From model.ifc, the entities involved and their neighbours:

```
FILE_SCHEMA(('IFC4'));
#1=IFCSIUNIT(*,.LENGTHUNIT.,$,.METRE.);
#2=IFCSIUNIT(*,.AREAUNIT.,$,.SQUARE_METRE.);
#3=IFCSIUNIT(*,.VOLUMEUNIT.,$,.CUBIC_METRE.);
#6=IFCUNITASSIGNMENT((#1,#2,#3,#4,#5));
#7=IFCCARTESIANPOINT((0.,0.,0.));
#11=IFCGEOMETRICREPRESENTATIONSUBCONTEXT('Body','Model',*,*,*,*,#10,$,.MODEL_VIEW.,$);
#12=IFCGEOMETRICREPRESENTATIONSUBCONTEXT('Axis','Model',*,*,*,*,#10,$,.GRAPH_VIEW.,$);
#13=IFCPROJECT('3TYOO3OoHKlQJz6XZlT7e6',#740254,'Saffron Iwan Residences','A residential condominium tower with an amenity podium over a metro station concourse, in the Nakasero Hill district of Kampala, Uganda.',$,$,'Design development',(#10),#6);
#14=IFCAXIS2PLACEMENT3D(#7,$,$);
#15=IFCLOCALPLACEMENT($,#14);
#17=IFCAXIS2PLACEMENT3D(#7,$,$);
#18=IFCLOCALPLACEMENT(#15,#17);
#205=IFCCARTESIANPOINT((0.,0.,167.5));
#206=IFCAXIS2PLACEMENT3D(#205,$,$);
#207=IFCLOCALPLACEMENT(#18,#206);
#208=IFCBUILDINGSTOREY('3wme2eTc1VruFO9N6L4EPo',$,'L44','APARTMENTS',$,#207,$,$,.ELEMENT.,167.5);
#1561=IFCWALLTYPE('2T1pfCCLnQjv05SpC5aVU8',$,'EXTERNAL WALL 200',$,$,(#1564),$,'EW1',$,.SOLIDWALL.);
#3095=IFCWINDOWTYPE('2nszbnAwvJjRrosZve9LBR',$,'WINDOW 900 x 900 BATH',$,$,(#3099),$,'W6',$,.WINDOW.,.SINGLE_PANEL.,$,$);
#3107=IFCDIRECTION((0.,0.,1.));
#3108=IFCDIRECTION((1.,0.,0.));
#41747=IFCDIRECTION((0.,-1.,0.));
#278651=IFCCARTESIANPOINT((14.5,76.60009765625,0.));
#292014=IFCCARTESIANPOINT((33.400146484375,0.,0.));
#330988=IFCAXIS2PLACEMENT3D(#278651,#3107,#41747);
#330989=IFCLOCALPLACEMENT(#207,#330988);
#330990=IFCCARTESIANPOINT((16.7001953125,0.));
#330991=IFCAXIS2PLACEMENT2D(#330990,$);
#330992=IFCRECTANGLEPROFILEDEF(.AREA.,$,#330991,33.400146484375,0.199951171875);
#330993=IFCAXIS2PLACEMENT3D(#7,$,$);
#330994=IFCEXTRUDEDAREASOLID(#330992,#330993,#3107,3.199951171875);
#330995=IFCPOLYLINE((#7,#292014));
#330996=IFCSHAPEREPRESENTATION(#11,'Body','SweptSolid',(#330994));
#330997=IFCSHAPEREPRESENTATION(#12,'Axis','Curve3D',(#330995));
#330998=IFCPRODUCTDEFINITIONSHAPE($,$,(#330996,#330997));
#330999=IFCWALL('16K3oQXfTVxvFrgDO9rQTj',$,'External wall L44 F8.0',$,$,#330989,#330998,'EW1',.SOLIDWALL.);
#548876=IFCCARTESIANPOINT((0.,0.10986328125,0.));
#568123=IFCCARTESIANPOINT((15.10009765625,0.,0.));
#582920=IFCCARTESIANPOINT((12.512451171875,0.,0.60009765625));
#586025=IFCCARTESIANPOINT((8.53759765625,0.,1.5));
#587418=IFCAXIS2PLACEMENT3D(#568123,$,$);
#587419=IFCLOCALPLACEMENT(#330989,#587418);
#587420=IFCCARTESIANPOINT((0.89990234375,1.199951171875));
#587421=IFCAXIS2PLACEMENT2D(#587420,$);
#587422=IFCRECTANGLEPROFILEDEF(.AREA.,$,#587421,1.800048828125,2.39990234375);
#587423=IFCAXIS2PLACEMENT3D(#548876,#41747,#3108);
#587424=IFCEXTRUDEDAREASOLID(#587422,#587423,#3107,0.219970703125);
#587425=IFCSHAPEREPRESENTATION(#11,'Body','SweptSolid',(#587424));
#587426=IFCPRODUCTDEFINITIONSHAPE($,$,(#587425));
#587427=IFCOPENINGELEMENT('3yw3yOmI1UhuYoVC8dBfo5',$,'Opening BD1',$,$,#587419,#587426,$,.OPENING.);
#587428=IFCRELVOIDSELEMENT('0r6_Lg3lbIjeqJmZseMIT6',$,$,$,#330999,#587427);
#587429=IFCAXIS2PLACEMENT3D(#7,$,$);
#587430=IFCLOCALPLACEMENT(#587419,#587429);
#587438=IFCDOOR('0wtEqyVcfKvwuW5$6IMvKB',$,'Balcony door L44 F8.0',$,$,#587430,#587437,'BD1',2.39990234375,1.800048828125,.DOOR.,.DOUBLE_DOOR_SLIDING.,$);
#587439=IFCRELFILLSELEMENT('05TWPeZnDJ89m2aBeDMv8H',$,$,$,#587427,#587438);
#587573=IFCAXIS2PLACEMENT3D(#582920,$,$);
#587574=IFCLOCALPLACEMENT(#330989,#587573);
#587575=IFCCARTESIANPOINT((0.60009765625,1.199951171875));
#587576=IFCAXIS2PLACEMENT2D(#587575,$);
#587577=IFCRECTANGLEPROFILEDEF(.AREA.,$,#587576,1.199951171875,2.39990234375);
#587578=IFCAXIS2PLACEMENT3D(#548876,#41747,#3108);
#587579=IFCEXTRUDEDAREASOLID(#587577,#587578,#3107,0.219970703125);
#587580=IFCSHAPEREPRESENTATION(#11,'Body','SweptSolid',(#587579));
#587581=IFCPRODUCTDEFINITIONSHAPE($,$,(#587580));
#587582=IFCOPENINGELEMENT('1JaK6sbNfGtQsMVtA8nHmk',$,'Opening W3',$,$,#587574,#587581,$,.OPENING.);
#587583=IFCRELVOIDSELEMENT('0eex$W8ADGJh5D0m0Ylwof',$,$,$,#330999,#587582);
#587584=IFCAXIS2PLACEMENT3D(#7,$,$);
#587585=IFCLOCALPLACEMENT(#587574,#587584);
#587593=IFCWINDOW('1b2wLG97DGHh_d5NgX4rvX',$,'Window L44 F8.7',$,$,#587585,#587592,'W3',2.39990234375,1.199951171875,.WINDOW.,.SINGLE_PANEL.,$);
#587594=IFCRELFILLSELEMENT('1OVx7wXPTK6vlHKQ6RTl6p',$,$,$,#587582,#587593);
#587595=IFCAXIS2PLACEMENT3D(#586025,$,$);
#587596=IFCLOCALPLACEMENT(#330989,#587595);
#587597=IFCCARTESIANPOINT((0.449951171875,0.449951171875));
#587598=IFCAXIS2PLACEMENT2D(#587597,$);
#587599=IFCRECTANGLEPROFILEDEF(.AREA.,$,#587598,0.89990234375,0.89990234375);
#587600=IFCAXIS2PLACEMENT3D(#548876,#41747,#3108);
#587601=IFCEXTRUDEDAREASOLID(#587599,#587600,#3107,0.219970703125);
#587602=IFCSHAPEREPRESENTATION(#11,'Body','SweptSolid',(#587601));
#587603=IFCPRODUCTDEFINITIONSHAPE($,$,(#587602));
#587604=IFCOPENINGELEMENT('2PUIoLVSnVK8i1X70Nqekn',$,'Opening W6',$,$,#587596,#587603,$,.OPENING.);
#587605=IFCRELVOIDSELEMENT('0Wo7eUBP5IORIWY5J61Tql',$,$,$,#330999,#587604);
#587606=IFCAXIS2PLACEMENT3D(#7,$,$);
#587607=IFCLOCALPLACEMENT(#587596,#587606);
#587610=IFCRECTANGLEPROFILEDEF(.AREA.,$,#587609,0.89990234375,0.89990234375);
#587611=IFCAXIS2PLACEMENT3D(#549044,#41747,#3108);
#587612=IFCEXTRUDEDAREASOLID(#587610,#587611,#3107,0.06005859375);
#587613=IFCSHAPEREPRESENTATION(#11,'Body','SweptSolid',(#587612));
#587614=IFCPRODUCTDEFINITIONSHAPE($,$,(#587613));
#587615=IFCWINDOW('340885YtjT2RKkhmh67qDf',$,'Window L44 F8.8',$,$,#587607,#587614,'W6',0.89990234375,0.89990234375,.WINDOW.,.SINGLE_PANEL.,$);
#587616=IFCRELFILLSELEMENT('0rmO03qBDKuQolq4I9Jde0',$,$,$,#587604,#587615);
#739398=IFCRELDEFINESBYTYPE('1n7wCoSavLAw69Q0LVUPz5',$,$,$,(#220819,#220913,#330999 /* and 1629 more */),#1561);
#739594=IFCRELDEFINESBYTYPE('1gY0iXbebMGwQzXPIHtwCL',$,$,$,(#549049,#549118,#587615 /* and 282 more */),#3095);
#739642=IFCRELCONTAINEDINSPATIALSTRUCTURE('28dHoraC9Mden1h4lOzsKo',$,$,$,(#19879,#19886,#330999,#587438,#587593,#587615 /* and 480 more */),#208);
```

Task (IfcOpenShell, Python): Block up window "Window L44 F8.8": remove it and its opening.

```python
import ifcopenshell
import ifcopenshell.api.feature
import ifcopenshell.api.root
import ifcopenshell.geom
import ifcopenshell.util.shape

model = ifcopenshell.open("model.ifc")
settings = ifcopenshell.geom.settings()


def volume(element):
    """Net volume in cubic metres, openings subtracted."""
    shape = ifcopenshell.geom.create_shape(settings, element)
    return ifcopenshell.util.shape.get_volume(shape.geometry)


window = model.by_id(587615)
opening = window.FillsVoids[0].RelatingOpeningElement
wall = opening.VoidsElements[0].RelatingBuildingElement
before = volume(wall)

ifcopenshell.api.root.remove_product(model, product=window)
ifcopenshell.api.feature.remove_feature(model, feature=opening)

after = volume(wall)

print(f"wall volume {before:.3f} -> {after:.3f} m3")

model.write("model_v2.ifc")
```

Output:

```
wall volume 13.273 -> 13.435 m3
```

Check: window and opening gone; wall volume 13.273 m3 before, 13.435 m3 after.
